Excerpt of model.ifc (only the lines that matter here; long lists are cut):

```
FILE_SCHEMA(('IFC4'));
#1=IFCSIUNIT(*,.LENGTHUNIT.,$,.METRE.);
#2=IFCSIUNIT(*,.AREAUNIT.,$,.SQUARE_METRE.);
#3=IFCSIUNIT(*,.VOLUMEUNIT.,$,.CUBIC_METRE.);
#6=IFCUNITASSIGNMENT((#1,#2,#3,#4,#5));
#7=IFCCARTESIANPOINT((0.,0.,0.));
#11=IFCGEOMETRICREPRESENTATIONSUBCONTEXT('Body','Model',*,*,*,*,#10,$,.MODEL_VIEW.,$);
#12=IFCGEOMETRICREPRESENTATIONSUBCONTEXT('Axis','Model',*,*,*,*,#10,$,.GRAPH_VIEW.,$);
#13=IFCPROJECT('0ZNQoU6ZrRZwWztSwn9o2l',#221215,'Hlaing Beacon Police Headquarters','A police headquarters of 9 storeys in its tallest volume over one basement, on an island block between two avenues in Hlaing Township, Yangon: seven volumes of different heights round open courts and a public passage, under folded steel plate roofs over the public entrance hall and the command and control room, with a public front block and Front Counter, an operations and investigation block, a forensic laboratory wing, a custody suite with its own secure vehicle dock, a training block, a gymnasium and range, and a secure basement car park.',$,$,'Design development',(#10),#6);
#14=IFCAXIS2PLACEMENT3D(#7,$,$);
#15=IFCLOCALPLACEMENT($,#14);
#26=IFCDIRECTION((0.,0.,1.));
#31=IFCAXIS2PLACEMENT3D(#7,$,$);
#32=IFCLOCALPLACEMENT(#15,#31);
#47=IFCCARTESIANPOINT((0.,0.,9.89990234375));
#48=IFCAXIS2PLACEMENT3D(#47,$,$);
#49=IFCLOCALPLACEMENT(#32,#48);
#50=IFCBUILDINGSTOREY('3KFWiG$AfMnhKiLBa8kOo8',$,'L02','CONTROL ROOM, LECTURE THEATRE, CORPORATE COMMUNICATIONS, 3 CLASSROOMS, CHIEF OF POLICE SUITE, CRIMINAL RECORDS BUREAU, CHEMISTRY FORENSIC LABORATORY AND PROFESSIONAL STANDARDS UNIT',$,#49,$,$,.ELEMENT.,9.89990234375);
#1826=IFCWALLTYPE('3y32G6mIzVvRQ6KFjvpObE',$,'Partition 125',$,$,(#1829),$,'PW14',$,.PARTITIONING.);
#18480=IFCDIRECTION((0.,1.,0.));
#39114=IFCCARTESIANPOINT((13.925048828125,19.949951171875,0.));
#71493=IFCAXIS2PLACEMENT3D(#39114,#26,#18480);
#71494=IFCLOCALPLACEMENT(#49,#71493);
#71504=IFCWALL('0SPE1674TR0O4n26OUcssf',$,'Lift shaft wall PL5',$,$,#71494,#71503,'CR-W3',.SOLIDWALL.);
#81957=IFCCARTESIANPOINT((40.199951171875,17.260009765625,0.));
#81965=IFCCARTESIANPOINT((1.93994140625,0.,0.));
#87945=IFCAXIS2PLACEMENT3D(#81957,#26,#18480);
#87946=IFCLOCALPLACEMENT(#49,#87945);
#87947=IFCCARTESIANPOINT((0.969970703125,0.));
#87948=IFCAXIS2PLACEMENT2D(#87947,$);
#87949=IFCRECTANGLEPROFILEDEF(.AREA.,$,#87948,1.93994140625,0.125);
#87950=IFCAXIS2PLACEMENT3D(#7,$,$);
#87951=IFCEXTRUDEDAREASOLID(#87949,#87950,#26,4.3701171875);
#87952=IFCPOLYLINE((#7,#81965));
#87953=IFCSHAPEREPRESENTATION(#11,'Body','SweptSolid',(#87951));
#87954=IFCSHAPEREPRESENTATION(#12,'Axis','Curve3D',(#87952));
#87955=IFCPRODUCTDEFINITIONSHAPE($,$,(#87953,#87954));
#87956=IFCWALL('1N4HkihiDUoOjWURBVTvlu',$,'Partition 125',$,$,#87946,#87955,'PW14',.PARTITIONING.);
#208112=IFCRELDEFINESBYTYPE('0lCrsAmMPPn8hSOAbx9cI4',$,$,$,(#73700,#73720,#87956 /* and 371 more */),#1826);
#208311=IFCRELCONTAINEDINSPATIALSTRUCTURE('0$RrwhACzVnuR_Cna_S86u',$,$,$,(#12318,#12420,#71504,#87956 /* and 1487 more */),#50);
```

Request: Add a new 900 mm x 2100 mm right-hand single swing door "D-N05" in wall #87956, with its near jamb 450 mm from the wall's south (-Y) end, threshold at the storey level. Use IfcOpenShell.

```python
import numpy as np
import ifcopenshell
import ifcopenshell.api.feature
import ifcopenshell.api.geometry
import ifcopenshell.api.root
import ifcopenshell.api.spatial
import ifcopenshell.geom
import ifcopenshell.util.element
import ifcopenshell.util.placement
import ifcopenshell.util.representation
import ifcopenshell.util.shape
import ifcopenshell.util.unit

model = ifcopenshell.open("model.ifc")
unit_scale = ifcopenshell.util.unit.calculate_unit_scale(model)
settings = ifcopenshell.geom.settings()


def volume(element):
    """Net volume in cubic metres, openings subtracted."""
    shape = ifcopenshell.geom.create_shape(settings, element)
    return ifcopenshell.util.shape.get_volume(shape.geometry)


wall = model.by_id(87956)
storey = ifcopenshell.util.element.get_container(wall, ifc_class="IfcBuildingStorey")
context = ifcopenshell.util.representation.get_context(model, "Model", "Body", "MODEL_VIEW")
before = volume(wall)

width, height, from_end, sill = 0.9, 2.1, 0.45, 0.0  # metres

# The wall runs along its own X axis, and the end named is its -X end.
wall_shape = ifcopenshell.geom.create_shape(settings, wall)
x, y, z = ifcopenshell.util.shape.get_vertices(wall_shape.geometry).T
start = x.min() + from_end
face, thickness = float(y.min()), float(y.max() - y.min())
wall_matrix = ifcopenshell.util.placement.get_local_placement(wall.ObjectPlacement)
level = ifcopenshell.util.placement.get_local_placement(storey.ObjectPlacement)[2, 3]


def in_wall(x, y):
    """Placement at x, y metres in the wall's axes, at sill height."""
    matrix = wall_matrix.copy()
    matrix[:, 3] = wall_matrix @ np.array([x / unit_scale, y / unit_scale, 0.0, 1.0])
    matrix[2, 3] = level + sill / unit_scale
    return matrix


# Opening: a box that overshoots both wall faces by 50 mm.
opening = ifcopenshell.api.root.create_entity(model, ifc_class="IfcOpeningElement", predefined_type="OPENING")
box = ifcopenshell.api.geometry.add_wall_representation(
    model, context=context, length=width, height=height, thickness=thickness + 0.1
)
ifcopenshell.api.geometry.assign_representation(model, product=opening, representation=box)
ifcopenshell.api.geometry.edit_object_placement(model, product=opening, matrix=in_wall(start, face - 0.05), is_si=False)
ifcopenshell.api.feature.add_feature(model, feature=opening, element=wall)

door = ifcopenshell.api.root.create_entity(model, ifc_class="IfcDoor", name="D-N05", predefined_type="DOOR")
door.OverallWidth, door.OverallHeight = width / unit_scale, height / unit_scale
door.OperationType = "SINGLE_SWING_RIGHT"
body = ifcopenshell.api.geometry.add_door_representation(
    model,
    context=context,
    overall_width=door.OverallWidth,
    overall_height=door.OverallHeight,
    operation_type="SINGLE_SWING_RIGHT",
    lining_properties={"LiningDepth": thickness / unit_scale, "ThresholdDepth": thickness / unit_scale},
)
ifcopenshell.api.geometry.assign_representation(model, product=door, representation=body)
ifcopenshell.api.spatial.assign_container(model, products=[door], relating_structure=storey)
ifcopenshell.api.feature.add_filling(model, opening=opening, element=door)

# The lining spans the wall, so the door starts at the wall face.
ifcopenshell.api.geometry.edit_object_placement(model, product=door, matrix=in_wall(start, face), is_si=False)

after = volume(wall)

print(f"wall volume {before:.3f} -> {after:.3f} m3")

model.write("model_edited.ifc")
```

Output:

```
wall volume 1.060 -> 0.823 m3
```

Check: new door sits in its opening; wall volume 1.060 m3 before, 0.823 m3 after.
